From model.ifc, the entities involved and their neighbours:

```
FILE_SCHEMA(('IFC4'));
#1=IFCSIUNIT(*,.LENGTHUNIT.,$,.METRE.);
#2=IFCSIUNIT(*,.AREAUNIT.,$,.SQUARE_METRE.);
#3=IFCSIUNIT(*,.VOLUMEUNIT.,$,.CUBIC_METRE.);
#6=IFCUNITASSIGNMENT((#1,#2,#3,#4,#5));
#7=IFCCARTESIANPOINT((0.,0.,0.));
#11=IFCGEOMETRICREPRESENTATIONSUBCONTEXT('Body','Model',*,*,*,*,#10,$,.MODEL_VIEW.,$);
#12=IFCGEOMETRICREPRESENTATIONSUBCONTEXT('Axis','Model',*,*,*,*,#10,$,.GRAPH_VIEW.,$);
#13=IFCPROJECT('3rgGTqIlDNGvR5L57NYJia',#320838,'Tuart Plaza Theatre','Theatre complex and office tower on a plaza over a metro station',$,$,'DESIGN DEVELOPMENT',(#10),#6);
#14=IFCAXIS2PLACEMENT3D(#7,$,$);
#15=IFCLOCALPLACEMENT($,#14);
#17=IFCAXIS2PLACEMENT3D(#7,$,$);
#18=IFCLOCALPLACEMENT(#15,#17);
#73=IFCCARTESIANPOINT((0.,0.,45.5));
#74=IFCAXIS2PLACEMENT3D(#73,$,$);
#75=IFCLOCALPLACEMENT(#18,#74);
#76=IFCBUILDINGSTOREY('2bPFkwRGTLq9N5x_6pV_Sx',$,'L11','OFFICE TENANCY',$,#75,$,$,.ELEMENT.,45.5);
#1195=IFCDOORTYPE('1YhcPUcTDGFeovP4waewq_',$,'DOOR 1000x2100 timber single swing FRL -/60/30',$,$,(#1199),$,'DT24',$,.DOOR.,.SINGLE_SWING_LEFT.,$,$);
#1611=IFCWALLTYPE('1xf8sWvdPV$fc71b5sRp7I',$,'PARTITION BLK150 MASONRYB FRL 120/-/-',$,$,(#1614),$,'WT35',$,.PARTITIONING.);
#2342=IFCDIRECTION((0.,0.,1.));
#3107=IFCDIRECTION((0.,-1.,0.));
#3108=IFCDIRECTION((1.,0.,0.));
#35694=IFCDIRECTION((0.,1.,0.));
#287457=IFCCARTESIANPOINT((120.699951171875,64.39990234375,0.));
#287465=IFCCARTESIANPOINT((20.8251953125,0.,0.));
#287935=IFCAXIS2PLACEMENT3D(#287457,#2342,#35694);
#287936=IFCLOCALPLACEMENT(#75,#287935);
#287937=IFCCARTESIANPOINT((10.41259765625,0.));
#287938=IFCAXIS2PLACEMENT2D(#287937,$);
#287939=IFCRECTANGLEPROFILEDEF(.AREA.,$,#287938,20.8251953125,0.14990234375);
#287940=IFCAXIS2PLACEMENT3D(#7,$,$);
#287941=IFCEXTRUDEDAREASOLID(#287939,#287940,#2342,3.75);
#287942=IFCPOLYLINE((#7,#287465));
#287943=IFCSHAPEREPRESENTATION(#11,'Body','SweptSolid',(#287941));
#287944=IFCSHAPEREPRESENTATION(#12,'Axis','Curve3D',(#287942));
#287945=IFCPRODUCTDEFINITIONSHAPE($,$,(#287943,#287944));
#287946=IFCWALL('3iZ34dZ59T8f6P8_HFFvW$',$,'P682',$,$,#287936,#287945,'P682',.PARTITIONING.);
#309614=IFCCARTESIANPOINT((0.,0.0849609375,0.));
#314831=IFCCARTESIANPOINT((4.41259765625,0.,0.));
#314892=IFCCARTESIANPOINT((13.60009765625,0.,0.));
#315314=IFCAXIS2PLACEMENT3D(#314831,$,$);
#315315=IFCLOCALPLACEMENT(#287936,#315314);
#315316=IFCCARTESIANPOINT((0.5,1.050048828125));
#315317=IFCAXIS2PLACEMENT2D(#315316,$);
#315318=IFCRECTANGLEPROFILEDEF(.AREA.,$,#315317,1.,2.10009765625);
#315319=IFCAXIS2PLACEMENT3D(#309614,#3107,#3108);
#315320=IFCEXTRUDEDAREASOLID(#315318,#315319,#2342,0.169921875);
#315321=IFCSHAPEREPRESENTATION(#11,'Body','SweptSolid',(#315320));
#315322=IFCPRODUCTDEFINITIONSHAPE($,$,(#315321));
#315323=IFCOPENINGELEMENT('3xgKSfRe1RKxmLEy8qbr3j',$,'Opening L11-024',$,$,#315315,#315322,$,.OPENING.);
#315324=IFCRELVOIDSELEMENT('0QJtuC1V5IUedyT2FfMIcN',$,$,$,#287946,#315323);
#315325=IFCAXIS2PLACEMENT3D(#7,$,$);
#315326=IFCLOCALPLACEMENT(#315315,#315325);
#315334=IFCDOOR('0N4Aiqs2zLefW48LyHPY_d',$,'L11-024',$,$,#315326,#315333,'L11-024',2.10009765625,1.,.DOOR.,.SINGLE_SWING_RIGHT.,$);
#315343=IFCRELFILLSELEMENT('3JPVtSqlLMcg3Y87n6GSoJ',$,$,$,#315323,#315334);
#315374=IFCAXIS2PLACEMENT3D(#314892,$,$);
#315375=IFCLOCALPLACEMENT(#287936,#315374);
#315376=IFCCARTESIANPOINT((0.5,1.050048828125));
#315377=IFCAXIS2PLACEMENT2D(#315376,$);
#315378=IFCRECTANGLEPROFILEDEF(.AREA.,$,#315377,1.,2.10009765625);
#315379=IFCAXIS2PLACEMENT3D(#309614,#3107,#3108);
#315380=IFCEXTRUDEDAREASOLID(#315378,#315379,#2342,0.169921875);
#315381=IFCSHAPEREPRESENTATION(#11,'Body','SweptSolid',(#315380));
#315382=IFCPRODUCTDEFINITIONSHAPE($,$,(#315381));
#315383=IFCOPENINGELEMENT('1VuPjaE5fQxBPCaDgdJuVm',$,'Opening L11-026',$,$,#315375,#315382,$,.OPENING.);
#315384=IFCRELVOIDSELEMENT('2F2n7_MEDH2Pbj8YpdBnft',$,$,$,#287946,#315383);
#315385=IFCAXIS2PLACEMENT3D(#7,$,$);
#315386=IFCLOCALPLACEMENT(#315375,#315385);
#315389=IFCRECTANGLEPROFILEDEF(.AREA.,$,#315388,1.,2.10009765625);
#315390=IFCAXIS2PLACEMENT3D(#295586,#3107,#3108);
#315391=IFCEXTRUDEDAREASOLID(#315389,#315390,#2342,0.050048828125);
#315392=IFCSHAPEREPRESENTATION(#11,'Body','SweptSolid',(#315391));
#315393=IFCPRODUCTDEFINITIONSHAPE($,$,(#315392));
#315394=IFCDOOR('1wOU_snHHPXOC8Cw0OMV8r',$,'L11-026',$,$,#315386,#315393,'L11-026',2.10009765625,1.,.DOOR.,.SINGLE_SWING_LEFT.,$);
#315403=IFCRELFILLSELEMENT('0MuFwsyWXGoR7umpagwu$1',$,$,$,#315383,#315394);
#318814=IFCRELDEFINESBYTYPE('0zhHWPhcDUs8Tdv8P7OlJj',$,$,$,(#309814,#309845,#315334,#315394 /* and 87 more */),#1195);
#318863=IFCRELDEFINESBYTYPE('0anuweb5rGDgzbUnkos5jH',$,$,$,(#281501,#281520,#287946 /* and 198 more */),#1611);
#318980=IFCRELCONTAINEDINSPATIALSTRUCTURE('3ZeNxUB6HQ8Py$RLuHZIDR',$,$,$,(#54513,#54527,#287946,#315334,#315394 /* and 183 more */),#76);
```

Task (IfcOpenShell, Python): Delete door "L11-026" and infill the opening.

```python
import ifcopenshell
import ifcopenshell.api.feature
import ifcopenshell.api.root
import ifcopenshell.geom
import ifcopenshell.util.shape

model = ifcopenshell.open("model.ifc")
settings = ifcopenshell.geom.settings()


def volume(element):
    """Net volume in cubic metres, openings subtracted."""
    shape = ifcopenshell.geom.create_shape(settings, element)
    return ifcopenshell.util.shape.get_volume(shape.geometry)


door = model.by_id(315394)
opening = door.FillsVoids[0].RelatingOpeningElement
wall = opening.VoidsElements[0].RelatingBuildingElement
before = volume(wall)

ifcopenshell.api.root.remove_product(model, product=door)
ifcopenshell.api.feature.remove_feature(model, feature=opening)

after = volume(wall)

print(f"wall volume {before:.3f} -> {after:.3f} m3")

model.write("model_updated.ifc")
```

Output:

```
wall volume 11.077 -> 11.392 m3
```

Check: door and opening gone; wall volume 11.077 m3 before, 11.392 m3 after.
